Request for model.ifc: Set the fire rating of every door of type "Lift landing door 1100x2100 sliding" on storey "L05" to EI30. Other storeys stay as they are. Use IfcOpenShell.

First a look at what the model holds.

```python
import ifcopenshell
import ifcopenshell.util.element

model = ifcopenshell.open("model.ifc")
print(model.schema)
storey = next(s for s in model.by_type("IfcBuildingStorey") if s.Name == "L05")
doors = [e for e in ifcopenshell.util.element.get_decomposition(storey) if e.is_a("IfcDoor")]
seen = {}
for e in doors:
    element_type = ifcopenshell.util.element.get_type(e)
    key = (element_type.Name if element_type != e and element_type else None, ifcopenshell.util.element.get_pset(e, "Pset_DoorCommon", "FireRating"))
    seen[key] = seen.get(key, 0) + 1
for (name, value), count in sorted(seen.items(), key=str):
    print(count, "x", name, "|", value)
```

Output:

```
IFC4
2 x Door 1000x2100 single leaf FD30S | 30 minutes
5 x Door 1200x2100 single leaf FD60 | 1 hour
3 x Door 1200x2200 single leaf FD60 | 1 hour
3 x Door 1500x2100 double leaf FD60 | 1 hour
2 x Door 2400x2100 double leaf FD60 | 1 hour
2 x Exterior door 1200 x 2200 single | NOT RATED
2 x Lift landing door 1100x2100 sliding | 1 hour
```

```python
import ifcopenshell
import ifcopenshell.api.pset
import ifcopenshell.util.element

model = ifcopenshell.open("model.ifc")

storey = next(s for s in model.by_type("IfcBuildingStorey") if s.Name == "L05")
doors = [e for e in ifcopenshell.util.element.get_decomposition(storey) if e.is_a("IfcDoor")]

count = 0
for e in doors:
    element_type = ifcopenshell.util.element.get_type(e)
    if element_type in (None, e) or element_type.Name != "Lift landing door 1100x2100 sliding":
        continue
    # add_pset returns the element's existing set when there is one.
    pset = ifcopenshell.api.pset.add_pset(model, product=e, name="Pset_DoorCommon")
    ifcopenshell.api.pset.edit_pset(model, pset=pset, properties={"FireRating": "EI30"})
    count += 1

print(count, "doors updated")

model.write("model_updated.ifc")
```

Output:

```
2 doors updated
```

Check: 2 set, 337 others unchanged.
